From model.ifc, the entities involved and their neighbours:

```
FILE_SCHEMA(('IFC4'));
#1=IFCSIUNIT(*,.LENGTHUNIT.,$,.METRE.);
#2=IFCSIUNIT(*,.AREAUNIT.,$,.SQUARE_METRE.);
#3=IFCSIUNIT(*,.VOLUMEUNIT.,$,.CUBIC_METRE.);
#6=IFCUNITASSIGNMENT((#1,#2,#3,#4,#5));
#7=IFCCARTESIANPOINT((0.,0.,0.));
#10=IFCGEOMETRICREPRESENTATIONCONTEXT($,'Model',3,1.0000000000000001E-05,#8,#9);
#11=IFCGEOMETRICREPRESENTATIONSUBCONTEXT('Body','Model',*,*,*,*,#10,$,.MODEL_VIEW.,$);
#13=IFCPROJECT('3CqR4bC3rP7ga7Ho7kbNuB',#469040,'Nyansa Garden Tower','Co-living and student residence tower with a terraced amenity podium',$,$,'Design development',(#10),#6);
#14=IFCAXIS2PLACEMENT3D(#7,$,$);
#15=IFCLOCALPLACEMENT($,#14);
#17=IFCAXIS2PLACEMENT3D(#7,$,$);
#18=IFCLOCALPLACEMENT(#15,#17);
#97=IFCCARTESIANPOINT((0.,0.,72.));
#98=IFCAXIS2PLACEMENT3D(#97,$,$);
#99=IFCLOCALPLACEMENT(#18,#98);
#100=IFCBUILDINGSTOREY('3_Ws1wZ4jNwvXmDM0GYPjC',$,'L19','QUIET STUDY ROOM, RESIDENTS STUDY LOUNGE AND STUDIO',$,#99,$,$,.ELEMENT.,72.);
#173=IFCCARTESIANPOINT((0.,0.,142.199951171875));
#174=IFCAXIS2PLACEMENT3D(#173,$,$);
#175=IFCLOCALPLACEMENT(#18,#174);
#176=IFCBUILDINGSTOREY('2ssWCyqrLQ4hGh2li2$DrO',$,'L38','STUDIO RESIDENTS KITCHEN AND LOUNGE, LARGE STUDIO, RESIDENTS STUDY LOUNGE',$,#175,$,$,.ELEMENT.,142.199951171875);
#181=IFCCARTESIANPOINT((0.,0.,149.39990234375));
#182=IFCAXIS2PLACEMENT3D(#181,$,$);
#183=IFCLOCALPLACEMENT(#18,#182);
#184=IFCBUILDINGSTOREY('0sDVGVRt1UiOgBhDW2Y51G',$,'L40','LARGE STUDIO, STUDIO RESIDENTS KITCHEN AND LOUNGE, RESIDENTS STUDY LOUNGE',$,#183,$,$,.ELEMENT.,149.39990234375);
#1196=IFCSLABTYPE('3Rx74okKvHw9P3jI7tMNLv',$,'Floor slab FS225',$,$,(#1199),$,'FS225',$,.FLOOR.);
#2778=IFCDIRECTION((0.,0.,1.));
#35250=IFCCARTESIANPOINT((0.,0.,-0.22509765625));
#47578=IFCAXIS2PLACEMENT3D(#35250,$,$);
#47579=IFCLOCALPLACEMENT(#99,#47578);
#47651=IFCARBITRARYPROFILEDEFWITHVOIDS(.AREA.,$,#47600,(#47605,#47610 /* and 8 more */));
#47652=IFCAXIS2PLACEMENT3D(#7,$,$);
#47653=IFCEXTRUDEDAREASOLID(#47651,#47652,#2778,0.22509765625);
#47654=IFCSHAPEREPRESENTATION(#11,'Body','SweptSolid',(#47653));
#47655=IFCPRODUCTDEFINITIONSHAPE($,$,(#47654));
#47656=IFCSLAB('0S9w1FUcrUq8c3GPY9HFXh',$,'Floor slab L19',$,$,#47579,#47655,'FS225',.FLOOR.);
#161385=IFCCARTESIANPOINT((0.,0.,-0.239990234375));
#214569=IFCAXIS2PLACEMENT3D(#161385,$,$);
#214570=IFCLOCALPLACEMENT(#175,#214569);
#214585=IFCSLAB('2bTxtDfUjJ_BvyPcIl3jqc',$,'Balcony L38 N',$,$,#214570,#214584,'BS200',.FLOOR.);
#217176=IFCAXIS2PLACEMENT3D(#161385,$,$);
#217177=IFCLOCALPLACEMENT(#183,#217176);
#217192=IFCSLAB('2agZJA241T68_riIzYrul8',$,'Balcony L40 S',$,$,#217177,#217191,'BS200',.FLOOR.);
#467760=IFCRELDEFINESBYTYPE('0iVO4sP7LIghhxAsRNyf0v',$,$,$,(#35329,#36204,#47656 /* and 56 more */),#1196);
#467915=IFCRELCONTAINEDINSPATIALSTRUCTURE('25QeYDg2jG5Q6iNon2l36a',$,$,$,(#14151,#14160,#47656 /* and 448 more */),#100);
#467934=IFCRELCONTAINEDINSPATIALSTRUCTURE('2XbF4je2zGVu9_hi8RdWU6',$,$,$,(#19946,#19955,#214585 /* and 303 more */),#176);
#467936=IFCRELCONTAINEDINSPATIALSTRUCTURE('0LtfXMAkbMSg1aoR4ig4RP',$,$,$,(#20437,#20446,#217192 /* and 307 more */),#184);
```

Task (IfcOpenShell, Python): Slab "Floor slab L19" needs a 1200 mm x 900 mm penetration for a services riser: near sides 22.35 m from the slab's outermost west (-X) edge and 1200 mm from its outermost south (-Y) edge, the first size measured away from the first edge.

```python
import numpy as np
import ifcopenshell
import ifcopenshell.api.feature
import ifcopenshell.api.geometry
import ifcopenshell.api.root
import ifcopenshell.geom
import ifcopenshell.util.placement
import ifcopenshell.util.representation
import ifcopenshell.util.shape
import ifcopenshell.util.unit

model = ifcopenshell.open("model.ifc")
unit_scale = ifcopenshell.util.unit.calculate_unit_scale(model)
settings = ifcopenshell.geom.settings()


def volume(element):
    """Net volume in cubic metres, openings subtracted."""
    shape = ifcopenshell.geom.create_shape(settings, element)
    return ifcopenshell.util.shape.get_volume(shape.geometry)


slab = model.by_id(47656)
before = volume(slab)

# Extent in the slab's own axes, in metres. The edges named are its -X and -Y sides.
slab_shape = ifcopenshell.geom.create_shape(settings, slab)
vertices = ifcopenshell.util.shape.get_vertices(slab_shape.geometry)
x_min, y_min, bottom = vertices.min(axis=0)
top = vertices[:, 2].max()

opening = ifcopenshell.api.root.create_entity(model, ifc_class="IfcOpeningElement", name="Services riser opening", predefined_type="OPENING")
context = ifcopenshell.util.representation.get_context(model, "Model", "Body", "MODEL_VIEW")
width, depth = 1.2, 0.9
outline = [(0.0, 0.0), (width, 0.0), (width, depth), (0.0, depth), (0.0, 0.0)]
# Overshoot both faces by 50 mm so the cut is clean.
shape = ifcopenshell.api.geometry.add_slab_representation(
    model, context=context, depth=top - bottom + 0.1, polyline=outline
)
ifcopenshell.api.geometry.assign_representation(model, product=opening, representation=shape)

matrix = ifcopenshell.util.placement.get_local_placement(slab.ObjectPlacement)
matrix[:, 3] = matrix @ np.append(np.array([x_min + 22.35, y_min + 1.2, bottom - 0.05]) / unit_scale, 1.0)
ifcopenshell.api.geometry.edit_object_placement(model, product=opening, matrix=matrix, is_si=False)
ifcopenshell.api.feature.add_feature(model, feature=opening, element=slab)

after = volume(slab)

print(f"slab volume {before:.3f} -> {after:.3f} m3")

model.write("model_v2.ifc")
```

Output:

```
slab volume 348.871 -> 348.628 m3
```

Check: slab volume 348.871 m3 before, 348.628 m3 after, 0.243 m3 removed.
